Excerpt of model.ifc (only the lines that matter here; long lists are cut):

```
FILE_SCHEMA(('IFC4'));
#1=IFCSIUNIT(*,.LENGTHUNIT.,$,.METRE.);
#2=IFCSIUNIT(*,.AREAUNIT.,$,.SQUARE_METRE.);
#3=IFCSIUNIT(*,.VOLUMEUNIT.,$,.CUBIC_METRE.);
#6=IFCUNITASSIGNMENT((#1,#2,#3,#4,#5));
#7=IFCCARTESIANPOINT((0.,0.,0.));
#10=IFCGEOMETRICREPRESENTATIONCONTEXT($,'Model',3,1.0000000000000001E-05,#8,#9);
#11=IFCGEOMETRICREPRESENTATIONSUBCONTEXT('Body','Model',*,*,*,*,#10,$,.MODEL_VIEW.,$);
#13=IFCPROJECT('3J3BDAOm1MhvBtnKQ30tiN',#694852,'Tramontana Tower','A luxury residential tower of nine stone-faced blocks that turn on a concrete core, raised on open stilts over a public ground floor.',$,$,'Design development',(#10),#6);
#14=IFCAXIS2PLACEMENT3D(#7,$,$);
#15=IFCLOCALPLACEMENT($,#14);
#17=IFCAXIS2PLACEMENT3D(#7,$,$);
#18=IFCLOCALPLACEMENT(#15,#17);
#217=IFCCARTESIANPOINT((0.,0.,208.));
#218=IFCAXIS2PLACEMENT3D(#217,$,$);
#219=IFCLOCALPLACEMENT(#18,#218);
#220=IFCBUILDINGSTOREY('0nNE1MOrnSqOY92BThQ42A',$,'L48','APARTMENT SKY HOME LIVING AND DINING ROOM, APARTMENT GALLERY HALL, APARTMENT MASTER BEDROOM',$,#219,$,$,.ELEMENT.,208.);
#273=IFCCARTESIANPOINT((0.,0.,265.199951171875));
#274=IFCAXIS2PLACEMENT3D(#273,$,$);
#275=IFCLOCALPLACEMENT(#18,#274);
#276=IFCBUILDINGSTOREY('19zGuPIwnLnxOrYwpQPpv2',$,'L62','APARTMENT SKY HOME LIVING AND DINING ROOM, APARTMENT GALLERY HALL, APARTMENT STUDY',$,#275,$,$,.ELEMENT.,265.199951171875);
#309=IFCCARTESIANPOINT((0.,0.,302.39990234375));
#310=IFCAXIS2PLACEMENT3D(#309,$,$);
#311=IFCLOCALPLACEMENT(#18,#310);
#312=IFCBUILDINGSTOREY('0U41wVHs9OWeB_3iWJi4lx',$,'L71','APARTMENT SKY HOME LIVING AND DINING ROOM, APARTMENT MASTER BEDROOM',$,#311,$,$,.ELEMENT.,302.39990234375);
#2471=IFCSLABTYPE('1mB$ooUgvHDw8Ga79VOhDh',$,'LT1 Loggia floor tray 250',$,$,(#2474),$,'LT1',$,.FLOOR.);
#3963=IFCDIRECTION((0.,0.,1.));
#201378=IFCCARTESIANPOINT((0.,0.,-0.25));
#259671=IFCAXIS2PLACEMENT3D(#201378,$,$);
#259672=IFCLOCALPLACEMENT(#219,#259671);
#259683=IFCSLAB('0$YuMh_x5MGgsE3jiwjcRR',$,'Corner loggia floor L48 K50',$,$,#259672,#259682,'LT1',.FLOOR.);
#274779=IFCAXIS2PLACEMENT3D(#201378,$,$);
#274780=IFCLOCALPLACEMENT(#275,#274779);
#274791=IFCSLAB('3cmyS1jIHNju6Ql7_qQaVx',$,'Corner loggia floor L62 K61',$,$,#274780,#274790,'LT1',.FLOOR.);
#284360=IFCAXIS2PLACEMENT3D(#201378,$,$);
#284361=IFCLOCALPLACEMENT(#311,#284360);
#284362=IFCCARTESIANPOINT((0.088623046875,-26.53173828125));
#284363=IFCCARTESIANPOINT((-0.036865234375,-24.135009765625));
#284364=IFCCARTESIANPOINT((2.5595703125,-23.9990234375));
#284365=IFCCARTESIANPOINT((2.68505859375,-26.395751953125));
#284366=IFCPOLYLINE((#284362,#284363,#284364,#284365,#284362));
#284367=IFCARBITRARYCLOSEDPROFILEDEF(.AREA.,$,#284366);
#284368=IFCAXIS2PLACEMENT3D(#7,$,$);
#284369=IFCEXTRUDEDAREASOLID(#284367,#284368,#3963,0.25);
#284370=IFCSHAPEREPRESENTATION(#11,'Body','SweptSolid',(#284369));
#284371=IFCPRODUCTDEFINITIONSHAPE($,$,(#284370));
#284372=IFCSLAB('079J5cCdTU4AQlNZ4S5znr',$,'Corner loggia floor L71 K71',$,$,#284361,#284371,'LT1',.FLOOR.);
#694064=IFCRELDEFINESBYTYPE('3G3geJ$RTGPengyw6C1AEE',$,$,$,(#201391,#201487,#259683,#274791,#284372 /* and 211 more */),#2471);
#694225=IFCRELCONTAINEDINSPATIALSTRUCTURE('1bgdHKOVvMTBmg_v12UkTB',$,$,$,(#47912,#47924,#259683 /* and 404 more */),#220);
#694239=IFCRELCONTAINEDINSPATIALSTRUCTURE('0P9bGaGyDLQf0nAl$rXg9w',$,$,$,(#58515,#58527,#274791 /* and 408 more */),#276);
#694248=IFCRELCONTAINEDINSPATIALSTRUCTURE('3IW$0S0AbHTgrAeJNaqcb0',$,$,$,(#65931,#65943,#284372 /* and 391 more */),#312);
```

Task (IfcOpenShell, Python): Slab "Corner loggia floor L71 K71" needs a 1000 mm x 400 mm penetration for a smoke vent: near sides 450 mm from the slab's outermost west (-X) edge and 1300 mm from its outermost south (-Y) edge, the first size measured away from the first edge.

```python
import numpy as np
import ifcopenshell
import ifcopenshell.api.feature
import ifcopenshell.api.geometry
import ifcopenshell.api.root
import ifcopenshell.geom
import ifcopenshell.util.placement
import ifcopenshell.util.representation
import ifcopenshell.util.shape
import ifcopenshell.util.unit

model = ifcopenshell.open("model.ifc")
unit_scale = ifcopenshell.util.unit.calculate_unit_scale(model)
settings = ifcopenshell.geom.settings()


def volume(element):
    """Net volume in cubic metres, openings subtracted."""
    shape = ifcopenshell.geom.create_shape(settings, element)
    return ifcopenshell.util.shape.get_volume(shape.geometry)


slab = model.by_guid("079J5cCdTU4AQlNZ4S5znr")
before = volume(slab)

# Extent in the slab's own axes, in metres. The edges named are its -X and -Y sides.
slab_shape = ifcopenshell.geom.create_shape(settings, slab)
vertices = ifcopenshell.util.shape.get_vertices(slab_shape.geometry)
x_min, y_min, bottom = vertices.min(axis=0)
top = vertices[:, 2].max()

opening = ifcopenshell.api.root.create_entity(model, ifc_class="IfcOpeningElement", name="Smoke vent opening", predefined_type="OPENING")
context = ifcopenshell.util.representation.get_context(model, "Model", "Body", "MODEL_VIEW")
width, depth = 1, 0.4
outline = [(0.0, 0.0), (width, 0.0), (width, depth), (0.0, depth), (0.0, 0.0)]
# Overshoot both faces by 50 mm so the cut is clean.
shape = ifcopenshell.api.geometry.add_slab_representation(
    model, context=context, depth=top - bottom + 0.1, polyline=outline
)
ifcopenshell.api.geometry.assign_representation(model, product=opening, representation=shape)

matrix = ifcopenshell.util.placement.get_local_placement(slab.ObjectPlacement)
matrix[:, 3] = matrix @ np.append(np.array([x_min + 0.45, y_min + 1.3, bottom - 0.05]) / unit_scale, 1.0)
ifcopenshell.api.geometry.edit_object_placement(model, product=opening, matrix=matrix, is_si=False)
ifcopenshell.api.feature.add_feature(model, feature=opening, element=slab)

after = volume(slab)

print(f"slab volume {before:.3f} -> {after:.3f} m3")

model.write("model_updated.ifc")
```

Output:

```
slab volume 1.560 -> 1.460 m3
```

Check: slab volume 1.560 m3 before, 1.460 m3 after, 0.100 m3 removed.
